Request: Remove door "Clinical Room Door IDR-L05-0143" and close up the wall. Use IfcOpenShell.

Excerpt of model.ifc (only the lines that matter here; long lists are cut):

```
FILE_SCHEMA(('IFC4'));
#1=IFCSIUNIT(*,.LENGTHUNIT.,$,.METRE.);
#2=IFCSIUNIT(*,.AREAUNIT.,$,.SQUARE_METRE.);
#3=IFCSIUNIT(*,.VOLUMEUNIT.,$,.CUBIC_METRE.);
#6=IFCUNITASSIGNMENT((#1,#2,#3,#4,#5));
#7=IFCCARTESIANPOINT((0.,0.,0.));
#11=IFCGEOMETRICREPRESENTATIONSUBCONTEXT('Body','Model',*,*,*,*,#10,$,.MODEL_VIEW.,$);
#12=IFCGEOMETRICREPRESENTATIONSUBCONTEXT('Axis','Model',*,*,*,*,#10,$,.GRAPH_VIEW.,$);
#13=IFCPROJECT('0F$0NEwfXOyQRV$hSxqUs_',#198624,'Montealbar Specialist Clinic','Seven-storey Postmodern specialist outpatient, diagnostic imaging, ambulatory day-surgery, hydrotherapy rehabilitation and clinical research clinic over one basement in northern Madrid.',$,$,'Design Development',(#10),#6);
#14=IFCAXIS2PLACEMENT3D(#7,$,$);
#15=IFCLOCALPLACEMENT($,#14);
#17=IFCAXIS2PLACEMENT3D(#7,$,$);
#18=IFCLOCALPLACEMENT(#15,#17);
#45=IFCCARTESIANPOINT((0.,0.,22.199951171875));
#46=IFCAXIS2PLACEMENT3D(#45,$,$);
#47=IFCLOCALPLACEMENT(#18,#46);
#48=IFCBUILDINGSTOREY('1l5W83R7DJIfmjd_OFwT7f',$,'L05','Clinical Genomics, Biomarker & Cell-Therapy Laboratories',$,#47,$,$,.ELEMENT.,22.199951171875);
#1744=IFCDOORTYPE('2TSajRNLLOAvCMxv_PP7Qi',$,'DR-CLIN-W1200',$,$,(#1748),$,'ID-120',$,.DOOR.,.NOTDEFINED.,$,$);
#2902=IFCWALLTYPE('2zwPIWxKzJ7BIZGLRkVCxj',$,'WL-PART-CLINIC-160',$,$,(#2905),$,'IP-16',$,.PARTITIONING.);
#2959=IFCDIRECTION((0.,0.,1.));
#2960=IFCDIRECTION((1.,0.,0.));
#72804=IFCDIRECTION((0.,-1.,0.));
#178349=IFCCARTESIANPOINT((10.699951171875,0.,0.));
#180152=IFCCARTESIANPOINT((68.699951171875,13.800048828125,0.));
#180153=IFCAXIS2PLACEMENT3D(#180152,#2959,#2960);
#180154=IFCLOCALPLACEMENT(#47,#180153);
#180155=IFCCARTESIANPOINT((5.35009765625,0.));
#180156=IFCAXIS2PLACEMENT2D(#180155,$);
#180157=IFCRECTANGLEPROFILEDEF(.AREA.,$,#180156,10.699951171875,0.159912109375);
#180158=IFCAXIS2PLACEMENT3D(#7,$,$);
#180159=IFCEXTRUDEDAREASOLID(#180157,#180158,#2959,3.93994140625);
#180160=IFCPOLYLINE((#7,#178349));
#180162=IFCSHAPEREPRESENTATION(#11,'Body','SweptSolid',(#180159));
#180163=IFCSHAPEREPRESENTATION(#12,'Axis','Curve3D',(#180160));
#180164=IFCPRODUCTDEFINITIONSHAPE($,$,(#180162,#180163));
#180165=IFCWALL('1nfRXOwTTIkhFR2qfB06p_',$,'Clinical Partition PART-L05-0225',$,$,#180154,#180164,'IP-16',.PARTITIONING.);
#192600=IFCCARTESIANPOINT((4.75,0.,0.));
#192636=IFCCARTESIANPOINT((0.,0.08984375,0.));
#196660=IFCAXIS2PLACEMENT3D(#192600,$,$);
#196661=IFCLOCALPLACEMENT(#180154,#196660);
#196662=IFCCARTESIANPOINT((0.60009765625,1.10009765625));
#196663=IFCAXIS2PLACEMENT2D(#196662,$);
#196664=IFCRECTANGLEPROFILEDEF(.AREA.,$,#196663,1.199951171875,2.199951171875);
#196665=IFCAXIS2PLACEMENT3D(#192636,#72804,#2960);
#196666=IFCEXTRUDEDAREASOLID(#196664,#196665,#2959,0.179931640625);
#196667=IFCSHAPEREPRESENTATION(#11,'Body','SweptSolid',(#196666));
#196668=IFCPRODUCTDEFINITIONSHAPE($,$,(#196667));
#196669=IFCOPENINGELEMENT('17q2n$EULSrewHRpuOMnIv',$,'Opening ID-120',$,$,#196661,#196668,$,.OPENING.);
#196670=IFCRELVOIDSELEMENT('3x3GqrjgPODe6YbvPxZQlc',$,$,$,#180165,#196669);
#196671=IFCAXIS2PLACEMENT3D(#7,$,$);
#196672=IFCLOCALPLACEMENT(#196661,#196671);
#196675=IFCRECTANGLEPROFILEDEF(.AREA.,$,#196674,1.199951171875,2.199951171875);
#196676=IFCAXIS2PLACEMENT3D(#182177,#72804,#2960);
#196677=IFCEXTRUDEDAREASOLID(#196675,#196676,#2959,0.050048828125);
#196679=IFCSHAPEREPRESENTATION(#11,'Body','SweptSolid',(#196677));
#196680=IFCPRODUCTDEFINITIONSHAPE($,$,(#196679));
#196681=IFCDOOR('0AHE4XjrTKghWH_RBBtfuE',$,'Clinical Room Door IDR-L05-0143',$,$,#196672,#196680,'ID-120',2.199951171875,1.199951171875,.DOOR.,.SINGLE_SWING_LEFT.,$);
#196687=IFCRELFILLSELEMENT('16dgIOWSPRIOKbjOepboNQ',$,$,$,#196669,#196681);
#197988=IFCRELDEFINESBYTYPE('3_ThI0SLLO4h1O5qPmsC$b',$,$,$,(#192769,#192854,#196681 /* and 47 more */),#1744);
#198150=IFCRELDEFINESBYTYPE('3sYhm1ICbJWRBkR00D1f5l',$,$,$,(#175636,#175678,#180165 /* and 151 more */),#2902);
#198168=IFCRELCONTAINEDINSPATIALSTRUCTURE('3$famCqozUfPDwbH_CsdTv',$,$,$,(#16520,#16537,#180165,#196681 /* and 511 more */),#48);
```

```python
import ifcopenshell
import ifcopenshell.api.feature
import ifcopenshell.api.root
import ifcopenshell.geom
import ifcopenshell.util.shape

model = ifcopenshell.open("model.ifc")
settings = ifcopenshell.geom.settings()


def volume(element):
    """Net volume in cubic metres, openings subtracted."""
    shape = ifcopenshell.geom.create_shape(settings, element)
    return ifcopenshell.util.shape.get_volume(shape.geometry)


door = model.by_guid("0AHE4XjrTKghWH_RBBtfuE")
opening = door.FillsVoids[0].RelatingOpeningElement
wall = opening.VoidsElements[0].RelatingBuildingElement
before = volume(wall)

ifcopenshell.api.root.remove_product(model, product=door)
ifcopenshell.api.feature.remove_feature(model, feature=opening)

after = volume(wall)

print(f"wall volume {before:.3f} -> {after:.3f} m3")

model.write("model_rev.ifc")
```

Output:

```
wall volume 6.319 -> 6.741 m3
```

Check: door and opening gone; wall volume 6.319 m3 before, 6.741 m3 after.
